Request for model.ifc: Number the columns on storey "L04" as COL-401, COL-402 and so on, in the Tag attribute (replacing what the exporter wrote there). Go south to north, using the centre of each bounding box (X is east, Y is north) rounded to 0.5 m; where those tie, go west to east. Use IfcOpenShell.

First a look at what the model holds.

```python
import ifcopenshell
import ifcopenshell.util.element
import ifcopenshell.util.placement

model = ifcopenshell.open("model.ifc")
print(model.schema)
storey = next(s for s in model.by_type("IfcBuildingStorey") if s.Name == "L04")
columns = [e for e in ifcopenshell.util.element.get_decomposition(storey) if e.is_a("IfcColumn")]
for e in sorted(columns, key=lambda e: e.id()):
    origin = ifcopenshell.util.placement.get_local_placement(e.ObjectPlacement)[:3, 3]
    print(e.id(), e.Tag, e.Name, origin.round(2) + 0.0, sep=" | ")
```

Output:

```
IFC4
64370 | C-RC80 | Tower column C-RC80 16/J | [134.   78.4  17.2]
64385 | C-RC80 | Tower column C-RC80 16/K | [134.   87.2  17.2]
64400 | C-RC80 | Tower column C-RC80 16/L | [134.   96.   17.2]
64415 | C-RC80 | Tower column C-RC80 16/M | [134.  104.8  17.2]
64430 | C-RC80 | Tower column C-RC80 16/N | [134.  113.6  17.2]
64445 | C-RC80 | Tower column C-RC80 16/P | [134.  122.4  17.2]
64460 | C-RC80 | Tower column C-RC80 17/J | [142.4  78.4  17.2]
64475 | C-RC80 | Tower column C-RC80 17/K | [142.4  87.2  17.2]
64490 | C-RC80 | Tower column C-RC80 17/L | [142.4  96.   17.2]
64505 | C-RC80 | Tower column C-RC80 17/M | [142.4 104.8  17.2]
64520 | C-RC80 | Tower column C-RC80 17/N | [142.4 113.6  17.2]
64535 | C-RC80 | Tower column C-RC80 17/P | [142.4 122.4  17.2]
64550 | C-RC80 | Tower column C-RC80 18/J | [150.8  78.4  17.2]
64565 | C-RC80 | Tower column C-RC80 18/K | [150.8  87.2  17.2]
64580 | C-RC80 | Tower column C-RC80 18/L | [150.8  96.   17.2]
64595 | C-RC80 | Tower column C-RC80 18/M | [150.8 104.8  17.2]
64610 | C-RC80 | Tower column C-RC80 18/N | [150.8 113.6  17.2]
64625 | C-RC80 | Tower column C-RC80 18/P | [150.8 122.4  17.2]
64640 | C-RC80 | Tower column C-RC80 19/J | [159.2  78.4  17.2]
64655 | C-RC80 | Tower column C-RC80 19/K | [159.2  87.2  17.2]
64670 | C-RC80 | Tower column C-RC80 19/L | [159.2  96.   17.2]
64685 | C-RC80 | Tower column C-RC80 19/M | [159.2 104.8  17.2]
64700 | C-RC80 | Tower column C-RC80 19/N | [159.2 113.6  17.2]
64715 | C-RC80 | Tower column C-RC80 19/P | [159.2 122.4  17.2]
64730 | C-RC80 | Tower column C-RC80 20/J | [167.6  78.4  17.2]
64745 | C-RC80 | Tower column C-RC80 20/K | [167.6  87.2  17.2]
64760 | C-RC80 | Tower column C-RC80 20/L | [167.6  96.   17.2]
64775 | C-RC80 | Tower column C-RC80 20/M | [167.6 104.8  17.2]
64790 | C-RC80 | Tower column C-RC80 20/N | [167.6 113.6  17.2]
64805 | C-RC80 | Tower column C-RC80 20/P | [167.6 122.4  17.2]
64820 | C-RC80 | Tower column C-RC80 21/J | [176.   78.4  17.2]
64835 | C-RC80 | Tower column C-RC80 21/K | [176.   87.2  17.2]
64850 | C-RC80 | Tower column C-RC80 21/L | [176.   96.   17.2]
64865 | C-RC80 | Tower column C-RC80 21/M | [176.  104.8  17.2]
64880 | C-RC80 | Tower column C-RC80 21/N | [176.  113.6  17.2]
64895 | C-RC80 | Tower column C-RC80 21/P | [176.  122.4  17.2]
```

```python
import ifcopenshell
import ifcopenshell.geom
import ifcopenshell.util.element
import ifcopenshell.util.shape

model = ifcopenshell.open("model.ifc")
settings = ifcopenshell.geom.settings()
settings.set("use-world-coords", True)


def centre(element):
    shape = ifcopenshell.geom.create_shape(settings, element)
    return ifcopenshell.util.shape.get_bbox_centroid(shape.geometry)


storey = next(s for s in model.by_type("IfcBuildingStorey") if s.Name == "L04")
columns = [e for e in ifcopenshell.util.element.get_decomposition(storey) if e.is_a("IfcColumn")]

# Insertion points can sit at a corner or the storey origin, so sort by the geometry (in metres).
centres = {e: centre(e) for e in columns}
columns.sort(key=lambda e: (round(centres[e][1] / 0.5), centres[e][0]))

for i, e in enumerate(columns, start=1):
    number = f"COL-4{i:02d}"
    e.Tag = number
    print(e.id(), number)

model.write("model_edited.ifc")
```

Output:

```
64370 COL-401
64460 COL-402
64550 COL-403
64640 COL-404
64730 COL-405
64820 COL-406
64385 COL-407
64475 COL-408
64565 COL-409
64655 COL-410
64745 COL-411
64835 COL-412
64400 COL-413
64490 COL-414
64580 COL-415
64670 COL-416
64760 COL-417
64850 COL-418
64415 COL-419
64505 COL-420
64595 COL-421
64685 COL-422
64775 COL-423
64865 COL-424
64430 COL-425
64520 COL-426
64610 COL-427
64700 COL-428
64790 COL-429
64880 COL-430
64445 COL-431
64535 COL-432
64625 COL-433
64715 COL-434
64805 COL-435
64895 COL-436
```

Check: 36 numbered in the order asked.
